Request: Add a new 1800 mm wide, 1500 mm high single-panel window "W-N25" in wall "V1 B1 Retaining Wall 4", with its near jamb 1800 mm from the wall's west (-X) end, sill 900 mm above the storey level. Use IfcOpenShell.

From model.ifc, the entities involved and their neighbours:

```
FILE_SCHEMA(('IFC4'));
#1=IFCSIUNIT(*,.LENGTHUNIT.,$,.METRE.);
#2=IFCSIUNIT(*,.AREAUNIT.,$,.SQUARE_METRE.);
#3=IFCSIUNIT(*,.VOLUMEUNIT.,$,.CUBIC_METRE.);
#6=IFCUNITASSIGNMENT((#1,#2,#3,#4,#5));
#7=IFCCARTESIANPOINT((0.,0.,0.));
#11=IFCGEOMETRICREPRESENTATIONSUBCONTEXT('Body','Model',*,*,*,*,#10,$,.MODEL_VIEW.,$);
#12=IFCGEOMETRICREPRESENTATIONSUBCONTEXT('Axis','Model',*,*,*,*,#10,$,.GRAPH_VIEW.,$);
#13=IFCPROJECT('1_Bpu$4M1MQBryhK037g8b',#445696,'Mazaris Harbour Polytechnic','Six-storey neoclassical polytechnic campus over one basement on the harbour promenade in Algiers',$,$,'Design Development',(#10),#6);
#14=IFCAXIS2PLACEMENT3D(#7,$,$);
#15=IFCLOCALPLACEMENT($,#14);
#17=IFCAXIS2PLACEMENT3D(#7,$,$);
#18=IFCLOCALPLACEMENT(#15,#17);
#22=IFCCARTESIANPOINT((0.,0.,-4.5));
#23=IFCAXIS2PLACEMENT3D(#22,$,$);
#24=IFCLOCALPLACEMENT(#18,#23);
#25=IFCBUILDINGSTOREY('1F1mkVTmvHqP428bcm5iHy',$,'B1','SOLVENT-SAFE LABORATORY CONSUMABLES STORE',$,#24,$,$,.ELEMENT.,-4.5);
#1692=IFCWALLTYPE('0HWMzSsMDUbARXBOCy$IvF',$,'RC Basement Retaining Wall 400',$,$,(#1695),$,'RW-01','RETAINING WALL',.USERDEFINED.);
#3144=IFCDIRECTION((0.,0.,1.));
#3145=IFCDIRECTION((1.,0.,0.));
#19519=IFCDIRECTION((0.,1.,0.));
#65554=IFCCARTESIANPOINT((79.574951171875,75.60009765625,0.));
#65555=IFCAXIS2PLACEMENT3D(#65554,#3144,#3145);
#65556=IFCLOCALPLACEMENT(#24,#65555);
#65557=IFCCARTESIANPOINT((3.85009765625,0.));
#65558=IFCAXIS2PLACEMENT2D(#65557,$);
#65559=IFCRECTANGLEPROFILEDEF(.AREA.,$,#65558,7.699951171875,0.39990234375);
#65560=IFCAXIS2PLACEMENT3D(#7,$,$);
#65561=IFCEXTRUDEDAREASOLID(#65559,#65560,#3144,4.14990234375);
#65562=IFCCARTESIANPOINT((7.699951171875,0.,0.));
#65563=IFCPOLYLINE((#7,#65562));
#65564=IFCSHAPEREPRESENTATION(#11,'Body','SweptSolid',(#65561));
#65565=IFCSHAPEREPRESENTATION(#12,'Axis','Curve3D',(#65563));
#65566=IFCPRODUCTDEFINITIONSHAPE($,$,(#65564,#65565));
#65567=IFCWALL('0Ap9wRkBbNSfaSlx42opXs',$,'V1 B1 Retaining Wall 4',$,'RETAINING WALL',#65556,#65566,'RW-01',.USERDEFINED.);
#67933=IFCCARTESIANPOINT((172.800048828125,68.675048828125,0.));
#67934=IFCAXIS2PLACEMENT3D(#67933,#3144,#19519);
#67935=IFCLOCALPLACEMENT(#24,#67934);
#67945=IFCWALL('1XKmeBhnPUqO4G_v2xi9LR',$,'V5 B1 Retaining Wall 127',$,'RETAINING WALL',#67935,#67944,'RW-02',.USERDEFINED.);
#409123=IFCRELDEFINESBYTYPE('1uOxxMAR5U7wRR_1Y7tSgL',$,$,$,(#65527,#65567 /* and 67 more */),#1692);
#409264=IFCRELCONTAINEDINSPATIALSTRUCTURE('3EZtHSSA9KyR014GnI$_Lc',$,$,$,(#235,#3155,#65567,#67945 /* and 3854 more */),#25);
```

```python
import numpy as np
import ifcopenshell
import ifcopenshell.api.feature
import ifcopenshell.api.geometry
import ifcopenshell.api.root
import ifcopenshell.api.spatial
import ifcopenshell.geom
import ifcopenshell.util.element
import ifcopenshell.util.placement
import ifcopenshell.util.representation
import ifcopenshell.util.shape
import ifcopenshell.util.unit

model = ifcopenshell.open("model.ifc")
unit_scale = ifcopenshell.util.unit.calculate_unit_scale(model)
settings = ifcopenshell.geom.settings()


def volume(element):
    """Net volume in cubic metres, openings subtracted."""
    shape = ifcopenshell.geom.create_shape(settings, element)
    return ifcopenshell.util.shape.get_volume(shape.geometry)


wall = model.by_id(65567)
storey = ifcopenshell.util.element.get_container(wall, ifc_class="IfcBuildingStorey")
context = ifcopenshell.util.representation.get_context(model, "Model", "Body", "MODEL_VIEW")
before = volume(wall)

width, height, from_end, sill = 1.8, 1.5, 1.8, 0.9  # metres

# The wall runs along its own X axis, and the end named is its -X end.
wall_shape = ifcopenshell.geom.create_shape(settings, wall)
x, y, z = ifcopenshell.util.shape.get_vertices(wall_shape.geometry).T
start = x.min() + from_end
face, thickness = float(y.min()), float(y.max() - y.min())
wall_matrix = ifcopenshell.util.placement.get_local_placement(wall.ObjectPlacement)
level = ifcopenshell.util.placement.get_local_placement(storey.ObjectPlacement)[2, 3]


def in_wall(x, y):
    """Placement at x, y metres in the wall's axes, at sill height."""
    matrix = wall_matrix.copy()
    matrix[:, 3] = wall_matrix @ np.array([x / unit_scale, y / unit_scale, 0.0, 1.0])
    matrix[2, 3] = level + sill / unit_scale
    return matrix


# Opening: a box that overshoots both wall faces by 50 mm.
opening = ifcopenshell.api.root.create_entity(model, ifc_class="IfcOpeningElement", predefined_type="OPENING")
box = ifcopenshell.api.geometry.add_wall_representation(
    model, context=context, length=width, height=height, thickness=thickness + 0.1
)
ifcopenshell.api.geometry.assign_representation(model, product=opening, representation=box)
ifcopenshell.api.geometry.edit_object_placement(model, product=opening, matrix=in_wall(start, face - 0.05), is_si=False)
ifcopenshell.api.feature.add_feature(model, feature=opening, element=wall)

window = ifcopenshell.api.root.create_entity(model, ifc_class="IfcWindow", name="W-N25", predefined_type="WINDOW")
window.OverallWidth, window.OverallHeight = width / unit_scale, height / unit_scale
window.PartitioningType = "SINGLE_PANEL"
body = ifcopenshell.api.geometry.add_window_representation(
    model,
    context=context,
    overall_width=window.OverallWidth,
    overall_height=window.OverallHeight,
    partition_type="SINGLE_PANEL",
)
ifcopenshell.api.geometry.assign_representation(model, product=window, representation=body)
ifcopenshell.api.spatial.assign_container(model, products=[window], relating_structure=storey)
ifcopenshell.api.feature.add_filling(model, opening=opening, element=window)

# Centre the window in the wall's thickness.
ifcopenshell.api.geometry.edit_object_placement(model, product=window, matrix=in_wall(start, face), is_si=False)
window_shape = ifcopenshell.geom.create_shape(settings, window)
depth = ifcopenshell.util.shape.get_vertices(window_shape.geometry)[:, 1]
offset = face + thickness / 2 - (depth.min() + depth.max()) / 2
ifcopenshell.api.geometry.edit_object_placement(model, product=window, matrix=in_wall(start, offset), is_si=False)

after = volume(wall)

print(f"wall volume {before:.3f} -> {after:.3f} m3")

model.write("model_rev.ifc")
```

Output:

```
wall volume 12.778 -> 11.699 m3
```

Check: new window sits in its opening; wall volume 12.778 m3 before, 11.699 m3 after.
